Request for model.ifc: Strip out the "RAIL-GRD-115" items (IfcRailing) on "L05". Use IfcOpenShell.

First a look at what the model holds.

```python
import ifcopenshell
import ifcopenshell.util.element

model = ifcopenshell.open("model.ifc")
print(model.schema)
storey = next(s for s in model.by_type("IfcBuildingStorey") if s.Name == "L05")
railings = [e for e in ifcopenshell.util.element.get_decomposition(storey) if e.is_a("IfcRailing")]
seen = {}
for e in railings:
    element_type = ifcopenshell.util.element.get_type(e)
    name = element_type.Name if element_type not in (None, e) else None
    seen[name] = seen.get(name, 0) + 1
for name, count in sorted(seen.items(), key=str):
    print(count, "x", name)
```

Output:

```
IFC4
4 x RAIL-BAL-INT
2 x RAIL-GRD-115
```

```python
import ifcopenshell
import ifcopenshell.api.root
import ifcopenshell.util.element

model = ifcopenshell.open("model.ifc")

storey = next(s for s in model.by_type("IfcBuildingStorey") if s.Name == "L05")
railings = [e for e in ifcopenshell.util.element.get_decomposition(storey) if e.is_a("IfcRailing")]
targets = [e for e in railings if (t := ifcopenshell.util.element.get_type(e)) not in (None, e) and t.Name == "RAIL-GRD-115"]

for e in targets:
    ifcopenshell.api.root.remove_product(model, product=e)
print(len(targets), "removed")

model.write("model_v2.ifc")
```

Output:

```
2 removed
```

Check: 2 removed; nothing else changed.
